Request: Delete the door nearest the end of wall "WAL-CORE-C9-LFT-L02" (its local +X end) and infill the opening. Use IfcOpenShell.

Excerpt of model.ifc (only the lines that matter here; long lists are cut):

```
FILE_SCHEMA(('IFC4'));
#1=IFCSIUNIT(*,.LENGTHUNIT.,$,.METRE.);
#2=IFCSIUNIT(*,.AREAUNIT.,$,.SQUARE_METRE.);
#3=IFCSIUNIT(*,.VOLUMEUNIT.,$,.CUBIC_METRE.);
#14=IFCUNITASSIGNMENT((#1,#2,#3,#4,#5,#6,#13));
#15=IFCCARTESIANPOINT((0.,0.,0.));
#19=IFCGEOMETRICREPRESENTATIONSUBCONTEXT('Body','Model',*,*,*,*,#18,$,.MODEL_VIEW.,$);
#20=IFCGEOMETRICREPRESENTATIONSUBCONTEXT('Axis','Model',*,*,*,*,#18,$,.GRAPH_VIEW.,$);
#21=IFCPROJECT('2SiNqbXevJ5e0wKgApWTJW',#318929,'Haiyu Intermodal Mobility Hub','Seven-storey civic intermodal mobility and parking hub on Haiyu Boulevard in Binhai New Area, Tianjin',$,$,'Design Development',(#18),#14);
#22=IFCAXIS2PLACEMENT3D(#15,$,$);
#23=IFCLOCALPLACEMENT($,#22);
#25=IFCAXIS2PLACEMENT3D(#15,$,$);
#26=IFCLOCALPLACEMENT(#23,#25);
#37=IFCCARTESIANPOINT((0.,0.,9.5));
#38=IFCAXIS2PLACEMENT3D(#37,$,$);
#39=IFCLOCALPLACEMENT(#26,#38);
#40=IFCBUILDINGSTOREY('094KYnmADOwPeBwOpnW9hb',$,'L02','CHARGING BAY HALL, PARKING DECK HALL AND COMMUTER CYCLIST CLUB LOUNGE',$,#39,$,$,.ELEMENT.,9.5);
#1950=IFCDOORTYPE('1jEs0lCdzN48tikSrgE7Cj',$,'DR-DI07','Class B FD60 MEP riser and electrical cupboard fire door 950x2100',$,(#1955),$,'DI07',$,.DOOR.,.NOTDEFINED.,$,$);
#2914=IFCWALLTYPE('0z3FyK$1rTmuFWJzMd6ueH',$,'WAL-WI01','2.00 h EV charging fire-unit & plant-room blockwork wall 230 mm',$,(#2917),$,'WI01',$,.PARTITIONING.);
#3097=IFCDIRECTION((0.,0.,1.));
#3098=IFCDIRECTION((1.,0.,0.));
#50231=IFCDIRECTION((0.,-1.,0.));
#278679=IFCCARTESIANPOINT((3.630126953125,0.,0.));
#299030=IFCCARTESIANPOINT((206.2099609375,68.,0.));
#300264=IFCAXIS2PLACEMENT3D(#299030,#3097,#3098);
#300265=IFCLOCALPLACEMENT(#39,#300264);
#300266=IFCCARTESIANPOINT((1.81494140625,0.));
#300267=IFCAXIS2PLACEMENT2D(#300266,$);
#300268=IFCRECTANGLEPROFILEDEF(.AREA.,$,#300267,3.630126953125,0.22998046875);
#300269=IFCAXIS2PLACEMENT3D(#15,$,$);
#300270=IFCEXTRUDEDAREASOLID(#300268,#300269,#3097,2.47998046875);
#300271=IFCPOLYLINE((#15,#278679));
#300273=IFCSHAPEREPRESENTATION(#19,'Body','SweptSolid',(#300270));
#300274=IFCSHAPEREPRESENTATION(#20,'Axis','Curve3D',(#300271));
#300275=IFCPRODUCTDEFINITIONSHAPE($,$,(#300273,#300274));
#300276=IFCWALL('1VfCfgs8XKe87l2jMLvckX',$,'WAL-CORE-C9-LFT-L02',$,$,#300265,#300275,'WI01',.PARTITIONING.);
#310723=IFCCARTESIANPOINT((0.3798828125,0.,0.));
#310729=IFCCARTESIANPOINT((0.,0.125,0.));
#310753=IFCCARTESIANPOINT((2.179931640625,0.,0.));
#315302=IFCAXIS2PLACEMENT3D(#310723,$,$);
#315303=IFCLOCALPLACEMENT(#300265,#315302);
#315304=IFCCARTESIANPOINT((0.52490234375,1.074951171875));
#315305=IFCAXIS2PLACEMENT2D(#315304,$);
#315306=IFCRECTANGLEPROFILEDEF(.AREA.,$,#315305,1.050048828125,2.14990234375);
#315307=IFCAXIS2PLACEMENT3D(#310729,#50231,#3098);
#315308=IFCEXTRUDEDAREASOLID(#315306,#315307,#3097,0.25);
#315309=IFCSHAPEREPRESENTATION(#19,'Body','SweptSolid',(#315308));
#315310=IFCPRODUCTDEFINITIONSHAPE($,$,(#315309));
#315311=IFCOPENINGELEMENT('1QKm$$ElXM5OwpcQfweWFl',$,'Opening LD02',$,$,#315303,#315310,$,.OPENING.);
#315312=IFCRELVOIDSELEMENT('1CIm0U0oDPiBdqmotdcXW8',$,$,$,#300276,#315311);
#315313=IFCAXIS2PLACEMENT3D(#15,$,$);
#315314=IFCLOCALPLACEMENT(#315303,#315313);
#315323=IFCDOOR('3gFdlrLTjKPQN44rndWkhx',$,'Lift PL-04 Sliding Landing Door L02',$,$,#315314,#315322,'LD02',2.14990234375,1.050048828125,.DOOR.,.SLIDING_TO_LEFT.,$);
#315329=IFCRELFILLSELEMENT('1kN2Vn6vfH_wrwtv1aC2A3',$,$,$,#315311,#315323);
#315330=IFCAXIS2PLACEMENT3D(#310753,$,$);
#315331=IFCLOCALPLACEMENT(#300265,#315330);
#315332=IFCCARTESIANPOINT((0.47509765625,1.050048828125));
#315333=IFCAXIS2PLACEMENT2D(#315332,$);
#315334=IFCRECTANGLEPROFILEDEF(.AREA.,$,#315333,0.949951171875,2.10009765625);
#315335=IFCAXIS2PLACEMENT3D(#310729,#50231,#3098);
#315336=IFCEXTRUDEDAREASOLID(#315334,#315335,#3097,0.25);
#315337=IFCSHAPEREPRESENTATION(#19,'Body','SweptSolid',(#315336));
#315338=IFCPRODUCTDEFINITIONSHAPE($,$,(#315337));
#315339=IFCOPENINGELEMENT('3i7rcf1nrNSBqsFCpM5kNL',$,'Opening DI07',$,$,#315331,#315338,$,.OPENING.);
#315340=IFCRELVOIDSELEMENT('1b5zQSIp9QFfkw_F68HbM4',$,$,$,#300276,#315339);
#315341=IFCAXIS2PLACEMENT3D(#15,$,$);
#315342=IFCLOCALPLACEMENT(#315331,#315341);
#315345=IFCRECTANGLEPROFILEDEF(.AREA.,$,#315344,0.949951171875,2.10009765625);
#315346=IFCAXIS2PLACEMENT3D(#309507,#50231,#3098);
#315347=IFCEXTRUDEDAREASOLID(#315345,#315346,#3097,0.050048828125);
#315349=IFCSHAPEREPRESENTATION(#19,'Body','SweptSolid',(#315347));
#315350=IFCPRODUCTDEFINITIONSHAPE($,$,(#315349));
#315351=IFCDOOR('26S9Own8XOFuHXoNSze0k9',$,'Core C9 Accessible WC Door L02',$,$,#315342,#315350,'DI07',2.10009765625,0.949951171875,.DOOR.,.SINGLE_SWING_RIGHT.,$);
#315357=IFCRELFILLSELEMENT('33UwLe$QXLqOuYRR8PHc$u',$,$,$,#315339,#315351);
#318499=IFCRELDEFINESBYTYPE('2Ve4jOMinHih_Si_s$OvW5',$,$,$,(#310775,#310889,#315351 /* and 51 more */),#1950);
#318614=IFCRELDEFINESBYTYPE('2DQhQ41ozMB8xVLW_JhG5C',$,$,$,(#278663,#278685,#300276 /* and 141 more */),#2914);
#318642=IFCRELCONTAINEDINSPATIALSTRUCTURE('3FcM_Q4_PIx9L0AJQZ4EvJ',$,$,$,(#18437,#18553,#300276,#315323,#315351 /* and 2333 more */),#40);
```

```python
import ifcopenshell
import ifcopenshell.api.feature
import ifcopenshell.api.root
import ifcopenshell.geom
import ifcopenshell.util.shape

model = ifcopenshell.open("model.ifc")
settings = ifcopenshell.geom.settings()


def volume(element):
    """Net volume in cubic metres, openings subtracted."""
    shape = ifcopenshell.geom.create_shape(settings, element)
    return ifcopenshell.util.shape.get_volume(shape.geometry)


door = model.by_guid("26S9Own8XOFuHXoNSze0k9")
opening = door.FillsVoids[0].RelatingOpeningElement
wall = opening.VoidsElements[0].RelatingBuildingElement
before = volume(wall)

ifcopenshell.api.root.remove_product(model, product=door)
ifcopenshell.api.feature.remove_feature(model, feature=opening)

after = volume(wall)

print(f"wall volume {before:.3f} -> {after:.3f} m3")

model.write("model_rev.ifc")
```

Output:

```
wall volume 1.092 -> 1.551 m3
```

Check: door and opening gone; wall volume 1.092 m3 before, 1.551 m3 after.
